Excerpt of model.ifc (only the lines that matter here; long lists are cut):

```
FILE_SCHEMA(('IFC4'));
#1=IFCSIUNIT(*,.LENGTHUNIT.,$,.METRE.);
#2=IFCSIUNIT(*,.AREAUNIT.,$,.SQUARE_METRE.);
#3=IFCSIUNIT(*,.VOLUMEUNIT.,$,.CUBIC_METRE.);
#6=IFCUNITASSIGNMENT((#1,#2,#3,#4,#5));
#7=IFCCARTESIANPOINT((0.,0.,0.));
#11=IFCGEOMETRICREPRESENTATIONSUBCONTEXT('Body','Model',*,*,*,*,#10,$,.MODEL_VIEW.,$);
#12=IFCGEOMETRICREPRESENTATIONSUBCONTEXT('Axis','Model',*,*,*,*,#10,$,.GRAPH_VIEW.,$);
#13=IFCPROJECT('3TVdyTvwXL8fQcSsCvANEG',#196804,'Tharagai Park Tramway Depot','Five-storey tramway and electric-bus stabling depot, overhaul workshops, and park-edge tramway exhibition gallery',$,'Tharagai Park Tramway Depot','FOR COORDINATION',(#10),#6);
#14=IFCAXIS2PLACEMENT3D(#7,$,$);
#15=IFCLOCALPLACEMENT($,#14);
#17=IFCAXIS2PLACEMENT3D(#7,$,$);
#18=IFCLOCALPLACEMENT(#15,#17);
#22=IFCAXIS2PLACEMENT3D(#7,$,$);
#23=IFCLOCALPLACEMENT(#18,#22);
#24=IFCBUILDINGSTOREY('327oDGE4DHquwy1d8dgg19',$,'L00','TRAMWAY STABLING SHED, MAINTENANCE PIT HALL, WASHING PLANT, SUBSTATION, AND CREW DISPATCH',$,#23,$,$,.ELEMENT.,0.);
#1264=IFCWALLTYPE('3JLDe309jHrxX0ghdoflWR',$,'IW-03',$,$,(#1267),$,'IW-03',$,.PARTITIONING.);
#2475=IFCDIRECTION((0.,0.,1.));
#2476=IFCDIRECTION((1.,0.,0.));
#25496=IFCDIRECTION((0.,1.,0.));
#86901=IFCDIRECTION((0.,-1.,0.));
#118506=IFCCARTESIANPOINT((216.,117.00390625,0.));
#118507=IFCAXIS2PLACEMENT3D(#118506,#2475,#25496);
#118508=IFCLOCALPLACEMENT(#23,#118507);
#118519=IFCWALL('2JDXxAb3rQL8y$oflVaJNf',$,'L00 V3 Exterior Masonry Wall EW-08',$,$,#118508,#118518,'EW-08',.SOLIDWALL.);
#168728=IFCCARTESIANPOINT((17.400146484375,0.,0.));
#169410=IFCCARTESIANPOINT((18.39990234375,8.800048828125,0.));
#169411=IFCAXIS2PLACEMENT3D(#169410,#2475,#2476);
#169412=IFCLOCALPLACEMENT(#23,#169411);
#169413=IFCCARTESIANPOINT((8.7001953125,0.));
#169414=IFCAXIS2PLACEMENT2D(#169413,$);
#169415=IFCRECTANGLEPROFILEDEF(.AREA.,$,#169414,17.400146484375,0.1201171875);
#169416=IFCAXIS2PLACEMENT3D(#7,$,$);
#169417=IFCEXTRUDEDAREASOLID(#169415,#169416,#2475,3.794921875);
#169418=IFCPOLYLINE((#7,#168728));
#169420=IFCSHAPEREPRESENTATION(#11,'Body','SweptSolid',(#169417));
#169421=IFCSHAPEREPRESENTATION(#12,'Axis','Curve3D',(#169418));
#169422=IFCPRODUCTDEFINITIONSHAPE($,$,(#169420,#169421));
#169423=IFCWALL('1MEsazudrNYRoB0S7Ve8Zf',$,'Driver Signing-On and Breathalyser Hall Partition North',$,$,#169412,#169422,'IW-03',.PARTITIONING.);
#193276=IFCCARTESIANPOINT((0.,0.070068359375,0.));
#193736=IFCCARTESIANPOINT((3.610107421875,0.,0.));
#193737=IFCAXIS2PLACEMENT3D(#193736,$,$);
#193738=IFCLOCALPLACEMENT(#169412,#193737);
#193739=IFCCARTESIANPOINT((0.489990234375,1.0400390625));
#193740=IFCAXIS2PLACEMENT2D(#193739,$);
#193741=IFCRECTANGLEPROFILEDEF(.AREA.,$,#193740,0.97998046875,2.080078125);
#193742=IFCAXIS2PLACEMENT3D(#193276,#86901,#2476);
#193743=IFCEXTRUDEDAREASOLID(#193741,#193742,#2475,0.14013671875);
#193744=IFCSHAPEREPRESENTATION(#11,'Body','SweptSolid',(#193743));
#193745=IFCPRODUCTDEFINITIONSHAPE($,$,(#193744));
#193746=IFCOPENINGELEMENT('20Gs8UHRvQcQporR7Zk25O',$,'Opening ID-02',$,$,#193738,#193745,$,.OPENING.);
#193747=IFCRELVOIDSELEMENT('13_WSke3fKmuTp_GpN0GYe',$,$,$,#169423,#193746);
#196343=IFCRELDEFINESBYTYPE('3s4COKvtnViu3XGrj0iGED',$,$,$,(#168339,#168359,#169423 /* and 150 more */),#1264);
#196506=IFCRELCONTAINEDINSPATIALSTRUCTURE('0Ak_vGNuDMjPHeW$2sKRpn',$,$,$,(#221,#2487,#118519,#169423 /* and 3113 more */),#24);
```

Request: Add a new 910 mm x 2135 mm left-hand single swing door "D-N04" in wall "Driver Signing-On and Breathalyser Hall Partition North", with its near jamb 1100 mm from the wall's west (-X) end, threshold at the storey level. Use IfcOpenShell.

```python
import numpy as np
import ifcopenshell
import ifcopenshell.api.feature
import ifcopenshell.api.geometry
import ifcopenshell.api.root
import ifcopenshell.api.spatial
import ifcopenshell.geom
import ifcopenshell.util.element
import ifcopenshell.util.placement
import ifcopenshell.util.representation
import ifcopenshell.util.shape
import ifcopenshell.util.unit

model = ifcopenshell.open("model.ifc")
unit_scale = ifcopenshell.util.unit.calculate_unit_scale(model)
settings = ifcopenshell.geom.settings()


def volume(element):
    """Net volume in cubic metres, openings subtracted."""
    shape = ifcopenshell.geom.create_shape(settings, element)
    return ifcopenshell.util.shape.get_volume(shape.geometry)


wall = model.by_guid("1MEsazudrNYRoB0S7Ve8Zf")
storey = ifcopenshell.util.element.get_container(wall, ifc_class="IfcBuildingStorey")
context = ifcopenshell.util.representation.get_context(model, "Model", "Body", "MODEL_VIEW")
before = volume(wall)

width, height, from_end, sill = 0.91, 2.135, 1.1, 0.0  # metres

# The wall runs along its own X axis, and the end named is its -X end.
wall_shape = ifcopenshell.geom.create_shape(settings, wall)
x, y, z = ifcopenshell.util.shape.get_vertices(wall_shape.geometry).T
start = x.min() + from_end
face, thickness = float(y.min()), float(y.max() - y.min())
wall_matrix = ifcopenshell.util.placement.get_local_placement(wall.ObjectPlacement)
level = ifcopenshell.util.placement.get_local_placement(storey.ObjectPlacement)[2, 3]


def in_wall(x, y):
    """Placement at x, y metres in the wall's axes, at sill height."""
    matrix = wall_matrix.copy()
    matrix[:, 3] = wall_matrix @ np.array([x / unit_scale, y / unit_scale, 0.0, 1.0])
    matrix[2, 3] = level + sill / unit_scale
    return matrix


# Opening: a box that overshoots both wall faces by 50 mm.
opening = ifcopenshell.api.root.create_entity(model, ifc_class="IfcOpeningElement", predefined_type="OPENING")
box = ifcopenshell.api.geometry.add_wall_representation(
    model, context=context, length=width, height=height, thickness=thickness + 0.1
)
ifcopenshell.api.geometry.assign_representation(model, product=opening, representation=box)
ifcopenshell.api.geometry.edit_object_placement(model, product=opening, matrix=in_wall(start, face - 0.05), is_si=False)
ifcopenshell.api.feature.add_feature(model, feature=opening, element=wall)

door = ifcopenshell.api.root.create_entity(model, ifc_class="IfcDoor", name="D-N04", predefined_type="DOOR")
door.OverallWidth, door.OverallHeight = width / unit_scale, height / unit_scale
door.OperationType = "SINGLE_SWING_LEFT"
body = ifcopenshell.api.geometry.add_door_representation(
    model,
    context=context,
    overall_width=door.OverallWidth,
    overall_height=door.OverallHeight,
    operation_type="SINGLE_SWING_LEFT",
    lining_properties={"LiningDepth": thickness / unit_scale, "ThresholdDepth": thickness / unit_scale},
)
ifcopenshell.api.geometry.assign_representation(model, product=door, representation=body)
ifcopenshell.api.spatial.assign_container(model, products=[door], relating_structure=storey)
ifcopenshell.api.feature.add_filling(model, opening=opening, element=door)

# The lining spans the wall, so the door starts at the wall face.
ifcopenshell.api.geometry.edit_object_placement(model, product=door, matrix=in_wall(start, face), is_si=False)

after = volume(wall)

print(f"wall volume {before:.3f} -> {after:.3f} m3")

model.write("model_v2.ifc")
```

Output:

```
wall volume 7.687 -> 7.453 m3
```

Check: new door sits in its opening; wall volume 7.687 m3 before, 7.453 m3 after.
